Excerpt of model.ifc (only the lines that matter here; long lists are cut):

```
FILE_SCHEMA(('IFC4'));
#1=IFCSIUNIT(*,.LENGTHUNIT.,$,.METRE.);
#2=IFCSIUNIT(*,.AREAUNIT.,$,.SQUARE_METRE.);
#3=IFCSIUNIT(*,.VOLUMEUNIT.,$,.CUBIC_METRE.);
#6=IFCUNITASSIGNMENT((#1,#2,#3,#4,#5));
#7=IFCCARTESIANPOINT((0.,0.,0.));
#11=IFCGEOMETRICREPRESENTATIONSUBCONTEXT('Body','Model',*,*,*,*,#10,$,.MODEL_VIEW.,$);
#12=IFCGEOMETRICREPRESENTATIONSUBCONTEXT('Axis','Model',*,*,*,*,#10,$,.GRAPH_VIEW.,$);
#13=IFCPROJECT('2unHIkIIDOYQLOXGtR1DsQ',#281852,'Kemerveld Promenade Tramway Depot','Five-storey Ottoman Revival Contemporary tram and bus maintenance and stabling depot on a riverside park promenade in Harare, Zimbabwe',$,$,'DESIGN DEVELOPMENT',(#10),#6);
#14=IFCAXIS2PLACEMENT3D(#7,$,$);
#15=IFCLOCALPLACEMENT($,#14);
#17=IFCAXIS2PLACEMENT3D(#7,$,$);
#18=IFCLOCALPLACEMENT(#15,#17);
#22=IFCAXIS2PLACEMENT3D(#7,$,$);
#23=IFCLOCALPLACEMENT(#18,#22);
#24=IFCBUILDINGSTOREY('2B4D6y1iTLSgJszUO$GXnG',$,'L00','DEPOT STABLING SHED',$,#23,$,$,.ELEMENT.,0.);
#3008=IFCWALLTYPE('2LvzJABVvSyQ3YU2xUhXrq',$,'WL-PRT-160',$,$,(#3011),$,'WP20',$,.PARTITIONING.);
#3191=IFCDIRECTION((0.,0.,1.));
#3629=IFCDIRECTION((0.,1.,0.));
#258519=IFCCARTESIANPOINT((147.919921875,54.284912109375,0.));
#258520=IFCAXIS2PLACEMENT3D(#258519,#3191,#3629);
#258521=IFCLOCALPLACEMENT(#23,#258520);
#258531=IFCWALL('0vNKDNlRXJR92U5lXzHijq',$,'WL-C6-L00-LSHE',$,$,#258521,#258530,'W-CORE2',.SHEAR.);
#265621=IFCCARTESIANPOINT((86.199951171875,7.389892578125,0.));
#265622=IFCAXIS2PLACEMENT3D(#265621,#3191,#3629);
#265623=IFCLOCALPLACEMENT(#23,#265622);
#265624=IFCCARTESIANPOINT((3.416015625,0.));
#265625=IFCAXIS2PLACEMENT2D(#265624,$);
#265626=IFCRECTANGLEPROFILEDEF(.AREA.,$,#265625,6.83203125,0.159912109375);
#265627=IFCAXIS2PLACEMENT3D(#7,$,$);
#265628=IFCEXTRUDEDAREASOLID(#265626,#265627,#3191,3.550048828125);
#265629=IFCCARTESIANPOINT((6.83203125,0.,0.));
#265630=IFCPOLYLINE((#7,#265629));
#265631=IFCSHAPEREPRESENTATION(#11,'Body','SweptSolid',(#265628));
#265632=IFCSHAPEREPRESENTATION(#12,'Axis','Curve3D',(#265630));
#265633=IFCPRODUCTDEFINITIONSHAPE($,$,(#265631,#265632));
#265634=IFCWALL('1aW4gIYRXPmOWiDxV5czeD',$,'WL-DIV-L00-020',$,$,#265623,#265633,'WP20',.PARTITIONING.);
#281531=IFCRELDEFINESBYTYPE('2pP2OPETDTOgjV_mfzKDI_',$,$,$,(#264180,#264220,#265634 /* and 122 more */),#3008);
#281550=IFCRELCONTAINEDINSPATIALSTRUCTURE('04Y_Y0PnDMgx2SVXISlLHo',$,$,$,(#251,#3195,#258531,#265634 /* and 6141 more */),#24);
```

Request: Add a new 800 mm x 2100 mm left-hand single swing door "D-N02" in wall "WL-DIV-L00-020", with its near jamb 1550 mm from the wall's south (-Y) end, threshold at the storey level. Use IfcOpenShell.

```python
import numpy as np
import ifcopenshell
import ifcopenshell.api.feature
import ifcopenshell.api.geometry
import ifcopenshell.api.root
import ifcopenshell.api.spatial
import ifcopenshell.geom
import ifcopenshell.util.element
import ifcopenshell.util.placement
import ifcopenshell.util.representation
import ifcopenshell.util.shape
import ifcopenshell.util.unit

model = ifcopenshell.open("model.ifc")
unit_scale = ifcopenshell.util.unit.calculate_unit_scale(model)
settings = ifcopenshell.geom.settings()


def volume(element):
    """Net volume in cubic metres, openings subtracted."""
    shape = ifcopenshell.geom.create_shape(settings, element)
    return ifcopenshell.util.shape.get_volume(shape.geometry)


wall = model.by_guid("1aW4gIYRXPmOWiDxV5czeD")
storey = ifcopenshell.util.element.get_container(wall, ifc_class="IfcBuildingStorey")
context = ifcopenshell.util.representation.get_context(model, "Model", "Body", "MODEL_VIEW")
before = volume(wall)

width, height, from_end, sill = 0.8, 2.1, 1.55, 0.0  # metres

# The wall runs along its own X axis, and the end named is its -X end.
wall_shape = ifcopenshell.geom.create_shape(settings, wall)
x, y, z = ifcopenshell.util.shape.get_vertices(wall_shape.geometry).T
start = x.min() + from_end
face, thickness = float(y.min()), float(y.max() - y.min())
wall_matrix = ifcopenshell.util.placement.get_local_placement(wall.ObjectPlacement)
level = ifcopenshell.util.placement.get_local_placement(storey.ObjectPlacement)[2, 3]


def in_wall(x, y):
    """Placement at x, y metres in the wall's axes, at sill height."""
    matrix = wall_matrix.copy()
    matrix[:, 3] = wall_matrix @ np.array([x / unit_scale, y / unit_scale, 0.0, 1.0])
    matrix[2, 3] = level + sill / unit_scale
    return matrix


# Opening: a box that overshoots both wall faces by 50 mm.
opening = ifcopenshell.api.root.create_entity(model, ifc_class="IfcOpeningElement", predefined_type="OPENING")
box = ifcopenshell.api.geometry.add_wall_representation(
    model, context=context, length=width, height=height, thickness=thickness + 0.1
)
ifcopenshell.api.geometry.assign_representation(model, product=opening, representation=box)
ifcopenshell.api.geometry.edit_object_placement(model, product=opening, matrix=in_wall(start, face - 0.05), is_si=False)
ifcopenshell.api.feature.add_feature(model, feature=opening, element=wall)

door = ifcopenshell.api.root.create_entity(model, ifc_class="IfcDoor", name="D-N02", predefined_type="DOOR")
door.OverallWidth, door.OverallHeight = width / unit_scale, height / unit_scale
door.OperationType = "SINGLE_SWING_LEFT"
body = ifcopenshell.api.geometry.add_door_representation(
    model,
    context=context,
    overall_width=door.OverallWidth,
    overall_height=door.OverallHeight,
    operation_type="SINGLE_SWING_LEFT",
    lining_properties={"LiningDepth": thickness / unit_scale, "ThresholdDepth": thickness / unit_scale},
)
ifcopenshell.api.geometry.assign_representation(model, product=door, representation=body)
ifcopenshell.api.spatial.assign_container(model, products=[door], relating_structure=storey)
ifcopenshell.api.feature.add_filling(model, opening=opening, element=door)

# The lining spans the wall, so the door starts at the wall face.
ifcopenshell.api.geometry.edit_object_placement(model, product=door, matrix=in_wall(start, face), is_si=False)

after = volume(wall)

print(f"wall volume {before:.3f} -> {after:.3f} m3")

model.write("model_rev.ifc")
```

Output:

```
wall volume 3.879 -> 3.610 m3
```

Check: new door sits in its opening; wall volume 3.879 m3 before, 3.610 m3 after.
